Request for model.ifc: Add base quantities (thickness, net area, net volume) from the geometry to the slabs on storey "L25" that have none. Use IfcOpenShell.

First a look at what the model holds.

```python
import ifcopenshell
import ifcopenshell.util.element
import ifcopenshell.util.unit

model = ifcopenshell.open("model.ifc")
print(model.schema)
for unit_type in ("LENGTHUNIT", "AREAUNIT", "VOLUMEUNIT"):
    print(unit_type, ifcopenshell.util.unit.calculate_unit_scale(model, unit_type))
storey = next(s for s in model.by_type("IfcBuildingStorey") if s.Name == "L25")
slabs = [e for e in ifcopenshell.util.element.get_decomposition(storey) if e.is_a("IfcSlab")]
for e in sorted(slabs, key=lambda e: e.id()):
    print(e.id(), e.is_a(), e.Name, list(ifcopenshell.util.element.get_psets(e, qtos_only=True)), sep=" | ")
```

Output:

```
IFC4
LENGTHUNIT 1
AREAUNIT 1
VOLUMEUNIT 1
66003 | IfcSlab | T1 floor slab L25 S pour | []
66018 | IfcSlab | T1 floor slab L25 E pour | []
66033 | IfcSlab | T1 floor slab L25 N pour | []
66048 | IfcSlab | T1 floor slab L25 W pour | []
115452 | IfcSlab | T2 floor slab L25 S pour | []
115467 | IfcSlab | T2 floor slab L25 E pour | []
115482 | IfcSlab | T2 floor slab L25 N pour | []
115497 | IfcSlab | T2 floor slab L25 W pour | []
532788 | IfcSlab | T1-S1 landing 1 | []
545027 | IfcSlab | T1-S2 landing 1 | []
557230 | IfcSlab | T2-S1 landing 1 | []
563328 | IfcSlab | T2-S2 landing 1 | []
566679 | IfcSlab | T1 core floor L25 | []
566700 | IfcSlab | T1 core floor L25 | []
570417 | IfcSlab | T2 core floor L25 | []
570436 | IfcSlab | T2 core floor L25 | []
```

```python
import ifcopenshell
import ifcopenshell.api.pset
import ifcopenshell.geom
import ifcopenshell.util.element
import ifcopenshell.util.shape
import ifcopenshell.util.unit

model = ifcopenshell.open("model.ifc")
unit_scale = ifcopenshell.util.unit.calculate_unit_scale(model)
area_scale = ifcopenshell.util.unit.calculate_unit_scale(model, "AREAUNIT")
volume_scale = ifcopenshell.util.unit.calculate_unit_scale(model, "VOLUMEUNIT")
settings = ifcopenshell.geom.settings()

storey = next(s for s in model.by_type("IfcBuildingStorey") if s.Name == "L25")
slabs = [e for e in ifcopenshell.util.element.get_decomposition(storey) if e.is_a("IfcSlab")]

for e in sorted(slabs, key=lambda e: e.id()):
    if ifcopenshell.util.element.get_psets(e, qtos_only=True, should_inherit=False):
        continue
    # Geometry comes back in metres, in the element's own axes.
    shape = ifcopenshell.geom.create_shape(settings, e)
    values = {
        "Width": ifcopenshell.util.shape.get_z(shape.geometry) / unit_scale,
        "NetArea": ifcopenshell.util.shape.get_footprint_area(shape.geometry) / area_scale,
        "NetVolume": ifcopenshell.util.shape.get_volume(shape.geometry) / volume_scale,
    }
    qto = ifcopenshell.api.pset.add_qto(model, product=e, name="Qto_SlabBaseQuantities")
    ifcopenshell.api.pset.edit_qto(model, qto=qto, properties=values)
    print(e.id(), {k: round(v, 3) for k, v in values.items()})

model.write("model_edited.ifc")
```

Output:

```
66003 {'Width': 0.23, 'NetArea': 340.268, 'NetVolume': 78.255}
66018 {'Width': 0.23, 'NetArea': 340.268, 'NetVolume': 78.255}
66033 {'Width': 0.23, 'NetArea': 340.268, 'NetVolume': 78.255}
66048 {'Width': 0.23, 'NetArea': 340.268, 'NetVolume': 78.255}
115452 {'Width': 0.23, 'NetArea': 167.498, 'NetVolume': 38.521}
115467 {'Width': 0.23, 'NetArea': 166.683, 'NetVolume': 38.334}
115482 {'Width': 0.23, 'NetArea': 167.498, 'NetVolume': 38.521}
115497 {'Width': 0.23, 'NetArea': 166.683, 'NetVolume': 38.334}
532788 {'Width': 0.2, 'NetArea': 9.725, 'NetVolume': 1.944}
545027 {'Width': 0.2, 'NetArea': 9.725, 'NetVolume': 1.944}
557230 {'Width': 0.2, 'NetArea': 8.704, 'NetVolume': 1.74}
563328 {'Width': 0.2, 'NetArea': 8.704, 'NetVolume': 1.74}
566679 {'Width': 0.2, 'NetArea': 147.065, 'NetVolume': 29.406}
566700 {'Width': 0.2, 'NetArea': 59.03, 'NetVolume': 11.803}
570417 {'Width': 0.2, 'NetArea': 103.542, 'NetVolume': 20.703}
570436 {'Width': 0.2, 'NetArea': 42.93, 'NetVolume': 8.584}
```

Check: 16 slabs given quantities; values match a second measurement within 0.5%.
